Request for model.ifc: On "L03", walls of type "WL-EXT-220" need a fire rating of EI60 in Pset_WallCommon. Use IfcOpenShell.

First a look at what the model holds.

```python
import ifcopenshell
import ifcopenshell.util.element

model = ifcopenshell.open("model.ifc")
print(model.schema)
storey = next(s for s in model.by_type("IfcBuildingStorey") if s.Name == "L03")
walls = [e for e in ifcopenshell.util.element.get_decomposition(storey) if e.is_a("IfcWall")]
seen = {}
for e in walls:
    element_type = ifcopenshell.util.element.get_type(e)
    key = (element_type.Name if element_type != e and element_type else None, ifcopenshell.util.element.get_pset(e, "Pset_WallCommon", "FireRating"))
    seen[key] = seen.get(key, 0) + 1
for (name, value), count in sorted(seen.items(), key=str):
    print(count, "x", name, "|", value)
```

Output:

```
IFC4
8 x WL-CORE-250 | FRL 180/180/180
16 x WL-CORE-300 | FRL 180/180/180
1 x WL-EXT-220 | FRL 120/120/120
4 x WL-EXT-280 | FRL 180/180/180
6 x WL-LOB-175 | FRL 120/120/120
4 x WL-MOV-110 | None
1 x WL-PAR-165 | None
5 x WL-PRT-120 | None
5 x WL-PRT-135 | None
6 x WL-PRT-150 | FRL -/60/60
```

```python
import ifcopenshell
import ifcopenshell.api.pset
import ifcopenshell.util.element

model = ifcopenshell.open("model.ifc")

storey = next(s for s in model.by_type("IfcBuildingStorey") if s.Name == "L03")
walls = [e for e in ifcopenshell.util.element.get_decomposition(storey) if e.is_a("IfcWall")]

count = 0
for e in walls:
    element_type = ifcopenshell.util.element.get_type(e)
    if element_type in (None, e) or element_type.Name != "WL-EXT-220":
        continue
    # add_pset returns the element's existing set when there is one.
    pset = ifcopenshell.api.pset.add_pset(model, product=e, name="Pset_WallCommon")
    ifcopenshell.api.pset.edit_pset(model, pset=pset, properties={"FireRating": "EI60"})
    count += 1

print(count, "walls updated")

model.write("model_v2.ifc")
```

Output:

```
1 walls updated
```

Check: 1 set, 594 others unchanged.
